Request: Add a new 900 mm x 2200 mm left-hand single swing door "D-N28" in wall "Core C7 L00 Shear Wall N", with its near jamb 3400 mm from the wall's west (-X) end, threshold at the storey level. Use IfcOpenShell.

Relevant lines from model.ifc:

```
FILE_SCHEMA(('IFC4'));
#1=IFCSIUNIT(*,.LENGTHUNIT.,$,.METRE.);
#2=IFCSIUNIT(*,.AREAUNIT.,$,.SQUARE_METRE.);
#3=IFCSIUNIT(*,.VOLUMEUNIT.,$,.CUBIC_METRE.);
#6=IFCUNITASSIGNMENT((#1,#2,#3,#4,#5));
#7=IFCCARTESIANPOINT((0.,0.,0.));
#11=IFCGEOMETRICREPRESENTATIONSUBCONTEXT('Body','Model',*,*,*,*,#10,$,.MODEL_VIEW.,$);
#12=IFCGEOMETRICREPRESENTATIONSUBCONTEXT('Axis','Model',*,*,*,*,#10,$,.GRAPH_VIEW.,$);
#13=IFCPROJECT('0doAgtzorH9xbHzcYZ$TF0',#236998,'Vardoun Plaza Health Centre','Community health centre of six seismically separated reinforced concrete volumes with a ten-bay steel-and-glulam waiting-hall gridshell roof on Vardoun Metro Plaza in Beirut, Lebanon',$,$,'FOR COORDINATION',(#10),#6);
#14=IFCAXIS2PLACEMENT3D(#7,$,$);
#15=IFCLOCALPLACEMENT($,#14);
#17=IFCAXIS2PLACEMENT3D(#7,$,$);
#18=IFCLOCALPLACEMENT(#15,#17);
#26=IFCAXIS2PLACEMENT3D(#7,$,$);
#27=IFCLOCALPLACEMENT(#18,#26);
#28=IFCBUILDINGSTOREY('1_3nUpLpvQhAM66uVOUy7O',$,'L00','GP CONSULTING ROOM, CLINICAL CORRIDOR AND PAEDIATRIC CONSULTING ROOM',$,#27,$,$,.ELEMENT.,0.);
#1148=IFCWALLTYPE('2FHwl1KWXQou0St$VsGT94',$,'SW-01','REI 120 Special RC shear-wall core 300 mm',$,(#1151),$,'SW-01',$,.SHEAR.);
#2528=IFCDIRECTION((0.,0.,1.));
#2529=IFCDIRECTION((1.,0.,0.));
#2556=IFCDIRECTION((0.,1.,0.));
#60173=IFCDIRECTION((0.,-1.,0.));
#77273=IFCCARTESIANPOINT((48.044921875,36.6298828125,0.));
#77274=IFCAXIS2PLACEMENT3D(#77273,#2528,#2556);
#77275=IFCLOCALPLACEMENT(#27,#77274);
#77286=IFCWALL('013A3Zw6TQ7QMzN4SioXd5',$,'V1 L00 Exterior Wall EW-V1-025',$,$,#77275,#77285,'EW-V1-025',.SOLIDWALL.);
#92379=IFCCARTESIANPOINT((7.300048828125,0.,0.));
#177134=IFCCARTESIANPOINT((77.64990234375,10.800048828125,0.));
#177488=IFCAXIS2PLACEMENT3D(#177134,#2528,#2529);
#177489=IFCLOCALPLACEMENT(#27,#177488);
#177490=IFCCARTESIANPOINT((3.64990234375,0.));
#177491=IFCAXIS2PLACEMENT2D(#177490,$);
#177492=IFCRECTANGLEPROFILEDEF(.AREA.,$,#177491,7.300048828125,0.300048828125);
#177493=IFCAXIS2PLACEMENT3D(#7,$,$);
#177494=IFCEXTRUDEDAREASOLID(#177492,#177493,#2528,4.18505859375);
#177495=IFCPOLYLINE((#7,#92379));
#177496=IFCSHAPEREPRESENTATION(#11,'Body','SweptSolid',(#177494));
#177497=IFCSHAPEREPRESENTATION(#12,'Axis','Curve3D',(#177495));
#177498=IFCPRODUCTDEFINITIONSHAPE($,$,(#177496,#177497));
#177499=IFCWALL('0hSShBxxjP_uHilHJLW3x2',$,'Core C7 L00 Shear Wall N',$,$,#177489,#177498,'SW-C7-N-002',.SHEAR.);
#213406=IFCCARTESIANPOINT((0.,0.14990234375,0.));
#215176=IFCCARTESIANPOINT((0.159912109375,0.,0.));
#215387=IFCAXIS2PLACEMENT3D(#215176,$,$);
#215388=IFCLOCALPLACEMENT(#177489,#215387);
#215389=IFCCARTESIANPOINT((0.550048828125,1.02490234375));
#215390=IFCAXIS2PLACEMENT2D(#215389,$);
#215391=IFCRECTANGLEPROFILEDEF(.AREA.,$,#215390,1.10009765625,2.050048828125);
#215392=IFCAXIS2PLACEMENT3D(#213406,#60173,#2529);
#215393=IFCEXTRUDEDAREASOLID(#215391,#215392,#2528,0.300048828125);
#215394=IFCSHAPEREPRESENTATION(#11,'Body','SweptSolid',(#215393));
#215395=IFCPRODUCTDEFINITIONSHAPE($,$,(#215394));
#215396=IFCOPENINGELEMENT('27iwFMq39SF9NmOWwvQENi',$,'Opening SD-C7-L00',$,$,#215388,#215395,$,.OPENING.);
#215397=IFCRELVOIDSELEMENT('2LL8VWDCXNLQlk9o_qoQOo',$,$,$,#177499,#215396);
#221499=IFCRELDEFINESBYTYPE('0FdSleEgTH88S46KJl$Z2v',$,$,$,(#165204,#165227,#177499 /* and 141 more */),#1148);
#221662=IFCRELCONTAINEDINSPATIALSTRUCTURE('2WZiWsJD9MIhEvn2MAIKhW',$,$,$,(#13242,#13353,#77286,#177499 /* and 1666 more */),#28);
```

```python
import numpy as np
import ifcopenshell
import ifcopenshell.api.feature
import ifcopenshell.api.geometry
import ifcopenshell.api.root
import ifcopenshell.api.spatial
import ifcopenshell.geom
import ifcopenshell.util.element
import ifcopenshell.util.placement
import ifcopenshell.util.representation
import ifcopenshell.util.shape
import ifcopenshell.util.unit

model = ifcopenshell.open("model.ifc")
unit_scale = ifcopenshell.util.unit.calculate_unit_scale(model)
settings = ifcopenshell.geom.settings()


def volume(element):
    """Net volume in cubic metres, openings subtracted."""
    shape = ifcopenshell.geom.create_shape(settings, element)
    return ifcopenshell.util.shape.get_volume(shape.geometry)


wall = model.by_guid("0hSShBxxjP_uHilHJLW3x2")
storey = ifcopenshell.util.element.get_container(wall, ifc_class="IfcBuildingStorey")
context = ifcopenshell.util.representation.get_context(model, "Model", "Body", "MODEL_VIEW")
before = volume(wall)

width, height, from_end, sill = 0.9, 2.2, 3.4, 0.0  # metres

# The wall runs along its own X axis, and the end named is its -X end.
wall_shape = ifcopenshell.geom.create_shape(settings, wall)
x, y, z = ifcopenshell.util.shape.get_vertices(wall_shape.geometry).T
start = x.min() + from_end
face, thickness = float(y.min()), float(y.max() - y.min())
wall_matrix = ifcopenshell.util.placement.get_local_placement(wall.ObjectPlacement)
level = ifcopenshell.util.placement.get_local_placement(storey.ObjectPlacement)[2, 3]


def in_wall(x, y):
    """Placement at x, y metres in the wall's axes, at sill height."""
    matrix = wall_matrix.copy()
    matrix[:, 3] = wall_matrix @ np.array([x / unit_scale, y / unit_scale, 0.0, 1.0])
    matrix[2, 3] = level + sill / unit_scale
    return matrix


# Opening: a box that overshoots both wall faces by 50 mm.
opening = ifcopenshell.api.root.create_entity(model, ifc_class="IfcOpeningElement", predefined_type="OPENING")
box = ifcopenshell.api.geometry.add_wall_representation(
    model, context=context, length=width, height=height, thickness=thickness + 0.1
)
ifcopenshell.api.geometry.assign_representation(model, product=opening, representation=box)
ifcopenshell.api.geometry.edit_object_placement(model, product=opening, matrix=in_wall(start, face - 0.05), is_si=False)
ifcopenshell.api.feature.add_feature(model, feature=opening, element=wall)

door = ifcopenshell.api.root.create_entity(model, ifc_class="IfcDoor", name="D-N28", predefined_type="DOOR")
door.OverallWidth, door.OverallHeight = width / unit_scale, height / unit_scale
door.OperationType = "SINGLE_SWING_LEFT"
body = ifcopenshell.api.geometry.add_door_representation(
    model,
    context=context,
    overall_width=door.OverallWidth,
    overall_height=door.OverallHeight,
    operation_type="SINGLE_SWING_LEFT",
    lining_properties={"LiningDepth": thickness / unit_scale, "ThresholdDepth": thickness / unit_scale},
)
ifcopenshell.api.geometry.assign_representation(model, product=door, representation=body)
ifcopenshell.api.spatial.assign_container(model, products=[door], relating_structure=storey)
ifcopenshell.api.feature.add_filling(model, opening=opening, element=door)

# The lining spans the wall, so the door starts at the wall face.
ifcopenshell.api.geometry.edit_object_placement(model, product=door, matrix=in_wall(start, face), is_si=False)

after = volume(wall)

print(f"wall volume {before:.3f} -> {after:.3f} m3")

model.write("model_updated.ifc")
```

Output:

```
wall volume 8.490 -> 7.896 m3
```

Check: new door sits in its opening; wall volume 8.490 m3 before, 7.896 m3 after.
